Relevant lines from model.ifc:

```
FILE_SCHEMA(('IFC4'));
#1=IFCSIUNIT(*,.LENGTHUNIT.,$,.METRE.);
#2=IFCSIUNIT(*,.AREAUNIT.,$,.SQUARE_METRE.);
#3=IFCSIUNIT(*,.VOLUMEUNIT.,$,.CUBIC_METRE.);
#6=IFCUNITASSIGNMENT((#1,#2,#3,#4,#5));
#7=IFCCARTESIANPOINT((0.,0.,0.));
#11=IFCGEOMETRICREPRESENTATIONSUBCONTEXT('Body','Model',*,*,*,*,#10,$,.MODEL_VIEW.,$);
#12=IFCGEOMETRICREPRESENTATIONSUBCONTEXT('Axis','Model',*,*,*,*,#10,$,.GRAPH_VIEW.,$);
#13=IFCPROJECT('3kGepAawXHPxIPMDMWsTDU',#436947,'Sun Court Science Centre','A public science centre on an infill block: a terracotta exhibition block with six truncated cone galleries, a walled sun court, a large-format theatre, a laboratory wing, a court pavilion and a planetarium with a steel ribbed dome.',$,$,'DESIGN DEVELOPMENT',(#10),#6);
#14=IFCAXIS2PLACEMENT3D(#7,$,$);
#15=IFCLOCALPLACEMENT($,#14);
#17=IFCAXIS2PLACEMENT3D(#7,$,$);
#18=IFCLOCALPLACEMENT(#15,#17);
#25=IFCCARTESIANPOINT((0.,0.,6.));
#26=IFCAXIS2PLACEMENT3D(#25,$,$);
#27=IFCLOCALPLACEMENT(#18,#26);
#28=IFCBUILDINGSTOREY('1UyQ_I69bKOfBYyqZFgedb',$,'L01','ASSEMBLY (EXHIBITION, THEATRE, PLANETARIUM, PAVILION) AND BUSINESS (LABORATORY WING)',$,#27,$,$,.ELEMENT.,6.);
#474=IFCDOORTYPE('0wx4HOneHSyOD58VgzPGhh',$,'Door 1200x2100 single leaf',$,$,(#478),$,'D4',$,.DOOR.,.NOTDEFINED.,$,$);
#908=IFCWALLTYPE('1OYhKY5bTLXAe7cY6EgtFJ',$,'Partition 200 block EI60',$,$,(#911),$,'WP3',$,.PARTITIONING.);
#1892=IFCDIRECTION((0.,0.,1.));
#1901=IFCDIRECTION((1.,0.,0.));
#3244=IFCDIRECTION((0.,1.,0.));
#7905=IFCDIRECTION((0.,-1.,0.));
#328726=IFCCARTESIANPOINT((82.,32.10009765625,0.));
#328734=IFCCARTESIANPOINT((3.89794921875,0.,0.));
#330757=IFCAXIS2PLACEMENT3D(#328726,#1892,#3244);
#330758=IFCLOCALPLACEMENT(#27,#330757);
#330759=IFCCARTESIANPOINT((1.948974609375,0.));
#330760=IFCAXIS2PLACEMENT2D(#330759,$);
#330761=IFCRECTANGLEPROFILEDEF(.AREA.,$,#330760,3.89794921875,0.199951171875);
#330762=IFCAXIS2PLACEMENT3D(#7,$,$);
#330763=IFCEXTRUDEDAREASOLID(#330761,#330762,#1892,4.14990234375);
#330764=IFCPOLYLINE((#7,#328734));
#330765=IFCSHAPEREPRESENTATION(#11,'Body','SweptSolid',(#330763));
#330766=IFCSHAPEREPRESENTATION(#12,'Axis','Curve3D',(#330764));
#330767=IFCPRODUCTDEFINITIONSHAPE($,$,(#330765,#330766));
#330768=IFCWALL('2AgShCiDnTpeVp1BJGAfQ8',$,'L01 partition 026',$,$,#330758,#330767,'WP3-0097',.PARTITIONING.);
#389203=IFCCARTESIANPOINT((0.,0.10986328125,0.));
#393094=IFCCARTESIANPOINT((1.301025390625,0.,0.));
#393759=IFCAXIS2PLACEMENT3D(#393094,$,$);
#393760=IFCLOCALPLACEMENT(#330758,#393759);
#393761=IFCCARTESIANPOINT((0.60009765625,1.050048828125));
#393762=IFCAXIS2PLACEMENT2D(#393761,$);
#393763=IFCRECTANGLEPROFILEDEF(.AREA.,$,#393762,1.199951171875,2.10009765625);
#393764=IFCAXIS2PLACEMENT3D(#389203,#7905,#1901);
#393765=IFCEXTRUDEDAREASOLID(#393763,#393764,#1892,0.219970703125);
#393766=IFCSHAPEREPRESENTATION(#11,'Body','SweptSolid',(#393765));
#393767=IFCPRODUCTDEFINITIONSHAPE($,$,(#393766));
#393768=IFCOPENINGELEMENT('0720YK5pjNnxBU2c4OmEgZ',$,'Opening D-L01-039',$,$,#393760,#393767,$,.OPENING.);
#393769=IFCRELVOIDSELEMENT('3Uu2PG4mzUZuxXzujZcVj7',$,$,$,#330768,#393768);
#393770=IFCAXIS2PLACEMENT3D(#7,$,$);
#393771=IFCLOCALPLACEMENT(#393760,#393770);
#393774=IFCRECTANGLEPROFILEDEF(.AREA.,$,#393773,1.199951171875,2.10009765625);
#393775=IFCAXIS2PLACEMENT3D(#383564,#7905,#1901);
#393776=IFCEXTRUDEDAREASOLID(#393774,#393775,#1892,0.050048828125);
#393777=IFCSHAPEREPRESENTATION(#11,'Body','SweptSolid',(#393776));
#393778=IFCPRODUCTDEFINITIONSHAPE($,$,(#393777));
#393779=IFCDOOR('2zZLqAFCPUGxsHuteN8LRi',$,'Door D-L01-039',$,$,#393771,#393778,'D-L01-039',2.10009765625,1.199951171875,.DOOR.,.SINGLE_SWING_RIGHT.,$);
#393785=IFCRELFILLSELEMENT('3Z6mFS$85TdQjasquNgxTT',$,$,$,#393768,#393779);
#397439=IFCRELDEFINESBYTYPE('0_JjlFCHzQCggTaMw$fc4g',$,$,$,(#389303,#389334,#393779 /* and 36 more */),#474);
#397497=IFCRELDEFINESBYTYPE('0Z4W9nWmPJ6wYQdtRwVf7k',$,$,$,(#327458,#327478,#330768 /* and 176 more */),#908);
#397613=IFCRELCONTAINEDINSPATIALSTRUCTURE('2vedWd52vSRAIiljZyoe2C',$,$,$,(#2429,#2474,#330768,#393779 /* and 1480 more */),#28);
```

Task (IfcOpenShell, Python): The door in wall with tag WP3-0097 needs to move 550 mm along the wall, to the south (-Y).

```python
import ifcopenshell
import ifcopenshell.api.geometry
import ifcopenshell.util.placement
import ifcopenshell.util.unit

model = ifcopenshell.open("model.ifc")
unit_scale = ifcopenshell.util.unit.calculate_unit_scale(model)

door = model.by_guid("2zZLqAFCPUGxsHuteN8LRi")
opening = door.FillsVoids[0].RelatingOpeningElement
wall = opening.VoidsElements[0].RelatingBuildingElement

wall_matrix = ifcopenshell.util.placement.get_local_placement(wall.ObjectPlacement)
shift = wall_matrix[:3, 0] * -0.55 / unit_scale
before = ifcopenshell.util.placement.get_local_placement(door.ObjectPlacement)[:3, 3].copy()

# The door is placed relative to its opening, so it follows when the opening moves.
matrix = ifcopenshell.util.placement.get_local_placement(opening.ObjectPlacement)
matrix[:3, 3] += shift
ifcopenshell.api.geometry.edit_object_placement(
    model, product=opening, matrix=matrix, is_si=False, should_transform_children=True
)

after = ifcopenshell.util.placement.get_local_placement(door.ObjectPlacement)[:3, 3]
print("door moved by", (after - before).round(3) + 0.0)

model.write("model_rev.ifc")
```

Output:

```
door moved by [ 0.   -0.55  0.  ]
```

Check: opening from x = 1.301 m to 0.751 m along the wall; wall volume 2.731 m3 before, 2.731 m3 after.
